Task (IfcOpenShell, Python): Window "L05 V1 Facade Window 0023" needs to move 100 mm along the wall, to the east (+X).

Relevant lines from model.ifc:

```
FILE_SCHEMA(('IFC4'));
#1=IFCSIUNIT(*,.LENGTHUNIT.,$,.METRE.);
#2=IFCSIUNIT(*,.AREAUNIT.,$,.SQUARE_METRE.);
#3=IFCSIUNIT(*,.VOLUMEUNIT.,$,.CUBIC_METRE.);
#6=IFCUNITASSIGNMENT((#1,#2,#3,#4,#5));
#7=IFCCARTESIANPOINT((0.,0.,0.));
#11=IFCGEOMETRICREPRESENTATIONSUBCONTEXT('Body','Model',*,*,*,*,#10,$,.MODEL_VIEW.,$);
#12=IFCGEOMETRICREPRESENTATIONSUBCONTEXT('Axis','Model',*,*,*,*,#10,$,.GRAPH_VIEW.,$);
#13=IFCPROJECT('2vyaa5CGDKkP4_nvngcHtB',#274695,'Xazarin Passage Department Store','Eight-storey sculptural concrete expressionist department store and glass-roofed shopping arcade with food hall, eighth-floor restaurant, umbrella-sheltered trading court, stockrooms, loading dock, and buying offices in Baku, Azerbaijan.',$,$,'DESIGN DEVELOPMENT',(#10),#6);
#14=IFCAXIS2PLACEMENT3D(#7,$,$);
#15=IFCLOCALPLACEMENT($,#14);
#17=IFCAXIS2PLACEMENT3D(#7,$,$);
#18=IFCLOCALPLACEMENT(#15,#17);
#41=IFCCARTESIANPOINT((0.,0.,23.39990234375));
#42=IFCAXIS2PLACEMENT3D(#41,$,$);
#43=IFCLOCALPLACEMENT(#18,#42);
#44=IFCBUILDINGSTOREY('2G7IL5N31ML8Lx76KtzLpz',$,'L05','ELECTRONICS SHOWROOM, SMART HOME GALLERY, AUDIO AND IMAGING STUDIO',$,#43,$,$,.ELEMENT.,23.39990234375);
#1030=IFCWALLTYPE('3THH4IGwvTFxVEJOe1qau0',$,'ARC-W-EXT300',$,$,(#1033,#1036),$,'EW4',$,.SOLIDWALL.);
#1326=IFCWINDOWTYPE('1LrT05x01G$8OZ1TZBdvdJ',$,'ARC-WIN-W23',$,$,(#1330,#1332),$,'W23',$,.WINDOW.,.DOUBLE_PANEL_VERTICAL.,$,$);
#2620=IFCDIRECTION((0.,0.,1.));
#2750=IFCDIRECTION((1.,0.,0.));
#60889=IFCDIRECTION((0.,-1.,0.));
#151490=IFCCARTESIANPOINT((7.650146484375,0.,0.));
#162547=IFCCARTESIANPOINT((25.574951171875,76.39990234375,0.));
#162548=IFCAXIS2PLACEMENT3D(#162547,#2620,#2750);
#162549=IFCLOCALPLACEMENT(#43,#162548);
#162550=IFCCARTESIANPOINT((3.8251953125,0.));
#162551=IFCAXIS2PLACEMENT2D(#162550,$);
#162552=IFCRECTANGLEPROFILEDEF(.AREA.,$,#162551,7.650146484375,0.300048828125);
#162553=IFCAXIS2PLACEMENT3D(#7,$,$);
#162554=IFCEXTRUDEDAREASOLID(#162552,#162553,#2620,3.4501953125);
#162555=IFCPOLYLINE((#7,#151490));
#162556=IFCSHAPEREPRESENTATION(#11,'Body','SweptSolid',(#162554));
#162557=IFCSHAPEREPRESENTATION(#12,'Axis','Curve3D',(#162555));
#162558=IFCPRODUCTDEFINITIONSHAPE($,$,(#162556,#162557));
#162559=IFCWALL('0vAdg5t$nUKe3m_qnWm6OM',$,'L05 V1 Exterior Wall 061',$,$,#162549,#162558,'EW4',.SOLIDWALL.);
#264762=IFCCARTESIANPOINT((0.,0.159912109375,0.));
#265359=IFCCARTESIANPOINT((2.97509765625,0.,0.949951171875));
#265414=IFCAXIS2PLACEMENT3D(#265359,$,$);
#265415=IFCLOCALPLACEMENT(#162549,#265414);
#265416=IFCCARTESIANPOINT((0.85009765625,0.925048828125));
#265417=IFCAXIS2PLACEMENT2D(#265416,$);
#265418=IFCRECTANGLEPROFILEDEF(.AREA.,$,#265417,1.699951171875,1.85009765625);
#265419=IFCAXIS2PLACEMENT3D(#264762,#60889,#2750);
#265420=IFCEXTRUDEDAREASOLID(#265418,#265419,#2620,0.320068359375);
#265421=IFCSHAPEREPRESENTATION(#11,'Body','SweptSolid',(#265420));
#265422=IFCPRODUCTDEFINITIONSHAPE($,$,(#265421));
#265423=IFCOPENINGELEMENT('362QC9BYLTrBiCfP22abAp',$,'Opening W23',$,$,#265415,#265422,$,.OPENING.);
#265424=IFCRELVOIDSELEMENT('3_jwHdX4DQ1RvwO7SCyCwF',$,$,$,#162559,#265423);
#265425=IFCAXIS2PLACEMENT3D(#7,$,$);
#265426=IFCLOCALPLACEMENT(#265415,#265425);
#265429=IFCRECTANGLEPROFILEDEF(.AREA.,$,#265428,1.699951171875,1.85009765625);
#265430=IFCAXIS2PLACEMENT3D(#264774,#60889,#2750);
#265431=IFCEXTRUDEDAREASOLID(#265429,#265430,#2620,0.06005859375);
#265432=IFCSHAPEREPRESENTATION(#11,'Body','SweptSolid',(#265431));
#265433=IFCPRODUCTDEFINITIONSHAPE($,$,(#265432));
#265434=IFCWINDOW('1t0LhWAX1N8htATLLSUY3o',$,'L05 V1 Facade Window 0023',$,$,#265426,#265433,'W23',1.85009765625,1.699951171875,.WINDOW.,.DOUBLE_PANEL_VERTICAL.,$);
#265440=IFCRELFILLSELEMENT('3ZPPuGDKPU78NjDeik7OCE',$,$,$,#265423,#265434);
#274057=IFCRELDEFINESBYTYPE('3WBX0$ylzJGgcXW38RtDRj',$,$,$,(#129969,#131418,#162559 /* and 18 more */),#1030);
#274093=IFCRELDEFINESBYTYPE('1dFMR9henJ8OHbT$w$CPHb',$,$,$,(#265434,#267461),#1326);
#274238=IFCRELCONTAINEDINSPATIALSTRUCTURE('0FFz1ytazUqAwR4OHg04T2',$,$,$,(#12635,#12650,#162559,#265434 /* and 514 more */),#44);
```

```python
import ifcopenshell
import ifcopenshell.api.geometry
import ifcopenshell.util.placement

model = ifcopenshell.open("model.ifc")

window = model.by_guid("1t0LhWAX1N8htATLLSUY3o")
opening = window.FillsVoids[0].RelatingOpeningElement
wall = opening.VoidsElements[0].RelatingBuildingElement

wall_matrix = ifcopenshell.util.placement.get_local_placement(wall.ObjectPlacement)
shift = wall_matrix[:3, 0] * 0.1
before = ifcopenshell.util.placement.get_local_placement(window.ObjectPlacement)[:3, 3].copy()

# The window is placed relative to its opening, so it follows when the opening moves.
matrix = ifcopenshell.util.placement.get_local_placement(opening.ObjectPlacement)
matrix[:3, 3] += shift
ifcopenshell.api.geometry.edit_object_placement(
    model, product=opening, matrix=matrix, is_si=False, should_transform_children=True
)

after = ifcopenshell.util.placement.get_local_placement(window.ObjectPlacement)[:3, 3]
print("window moved by", (after - before).round(3) + 0.0)

model.write("model_v2.ifc")
```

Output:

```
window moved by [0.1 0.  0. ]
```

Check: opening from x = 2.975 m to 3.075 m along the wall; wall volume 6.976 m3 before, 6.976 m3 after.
